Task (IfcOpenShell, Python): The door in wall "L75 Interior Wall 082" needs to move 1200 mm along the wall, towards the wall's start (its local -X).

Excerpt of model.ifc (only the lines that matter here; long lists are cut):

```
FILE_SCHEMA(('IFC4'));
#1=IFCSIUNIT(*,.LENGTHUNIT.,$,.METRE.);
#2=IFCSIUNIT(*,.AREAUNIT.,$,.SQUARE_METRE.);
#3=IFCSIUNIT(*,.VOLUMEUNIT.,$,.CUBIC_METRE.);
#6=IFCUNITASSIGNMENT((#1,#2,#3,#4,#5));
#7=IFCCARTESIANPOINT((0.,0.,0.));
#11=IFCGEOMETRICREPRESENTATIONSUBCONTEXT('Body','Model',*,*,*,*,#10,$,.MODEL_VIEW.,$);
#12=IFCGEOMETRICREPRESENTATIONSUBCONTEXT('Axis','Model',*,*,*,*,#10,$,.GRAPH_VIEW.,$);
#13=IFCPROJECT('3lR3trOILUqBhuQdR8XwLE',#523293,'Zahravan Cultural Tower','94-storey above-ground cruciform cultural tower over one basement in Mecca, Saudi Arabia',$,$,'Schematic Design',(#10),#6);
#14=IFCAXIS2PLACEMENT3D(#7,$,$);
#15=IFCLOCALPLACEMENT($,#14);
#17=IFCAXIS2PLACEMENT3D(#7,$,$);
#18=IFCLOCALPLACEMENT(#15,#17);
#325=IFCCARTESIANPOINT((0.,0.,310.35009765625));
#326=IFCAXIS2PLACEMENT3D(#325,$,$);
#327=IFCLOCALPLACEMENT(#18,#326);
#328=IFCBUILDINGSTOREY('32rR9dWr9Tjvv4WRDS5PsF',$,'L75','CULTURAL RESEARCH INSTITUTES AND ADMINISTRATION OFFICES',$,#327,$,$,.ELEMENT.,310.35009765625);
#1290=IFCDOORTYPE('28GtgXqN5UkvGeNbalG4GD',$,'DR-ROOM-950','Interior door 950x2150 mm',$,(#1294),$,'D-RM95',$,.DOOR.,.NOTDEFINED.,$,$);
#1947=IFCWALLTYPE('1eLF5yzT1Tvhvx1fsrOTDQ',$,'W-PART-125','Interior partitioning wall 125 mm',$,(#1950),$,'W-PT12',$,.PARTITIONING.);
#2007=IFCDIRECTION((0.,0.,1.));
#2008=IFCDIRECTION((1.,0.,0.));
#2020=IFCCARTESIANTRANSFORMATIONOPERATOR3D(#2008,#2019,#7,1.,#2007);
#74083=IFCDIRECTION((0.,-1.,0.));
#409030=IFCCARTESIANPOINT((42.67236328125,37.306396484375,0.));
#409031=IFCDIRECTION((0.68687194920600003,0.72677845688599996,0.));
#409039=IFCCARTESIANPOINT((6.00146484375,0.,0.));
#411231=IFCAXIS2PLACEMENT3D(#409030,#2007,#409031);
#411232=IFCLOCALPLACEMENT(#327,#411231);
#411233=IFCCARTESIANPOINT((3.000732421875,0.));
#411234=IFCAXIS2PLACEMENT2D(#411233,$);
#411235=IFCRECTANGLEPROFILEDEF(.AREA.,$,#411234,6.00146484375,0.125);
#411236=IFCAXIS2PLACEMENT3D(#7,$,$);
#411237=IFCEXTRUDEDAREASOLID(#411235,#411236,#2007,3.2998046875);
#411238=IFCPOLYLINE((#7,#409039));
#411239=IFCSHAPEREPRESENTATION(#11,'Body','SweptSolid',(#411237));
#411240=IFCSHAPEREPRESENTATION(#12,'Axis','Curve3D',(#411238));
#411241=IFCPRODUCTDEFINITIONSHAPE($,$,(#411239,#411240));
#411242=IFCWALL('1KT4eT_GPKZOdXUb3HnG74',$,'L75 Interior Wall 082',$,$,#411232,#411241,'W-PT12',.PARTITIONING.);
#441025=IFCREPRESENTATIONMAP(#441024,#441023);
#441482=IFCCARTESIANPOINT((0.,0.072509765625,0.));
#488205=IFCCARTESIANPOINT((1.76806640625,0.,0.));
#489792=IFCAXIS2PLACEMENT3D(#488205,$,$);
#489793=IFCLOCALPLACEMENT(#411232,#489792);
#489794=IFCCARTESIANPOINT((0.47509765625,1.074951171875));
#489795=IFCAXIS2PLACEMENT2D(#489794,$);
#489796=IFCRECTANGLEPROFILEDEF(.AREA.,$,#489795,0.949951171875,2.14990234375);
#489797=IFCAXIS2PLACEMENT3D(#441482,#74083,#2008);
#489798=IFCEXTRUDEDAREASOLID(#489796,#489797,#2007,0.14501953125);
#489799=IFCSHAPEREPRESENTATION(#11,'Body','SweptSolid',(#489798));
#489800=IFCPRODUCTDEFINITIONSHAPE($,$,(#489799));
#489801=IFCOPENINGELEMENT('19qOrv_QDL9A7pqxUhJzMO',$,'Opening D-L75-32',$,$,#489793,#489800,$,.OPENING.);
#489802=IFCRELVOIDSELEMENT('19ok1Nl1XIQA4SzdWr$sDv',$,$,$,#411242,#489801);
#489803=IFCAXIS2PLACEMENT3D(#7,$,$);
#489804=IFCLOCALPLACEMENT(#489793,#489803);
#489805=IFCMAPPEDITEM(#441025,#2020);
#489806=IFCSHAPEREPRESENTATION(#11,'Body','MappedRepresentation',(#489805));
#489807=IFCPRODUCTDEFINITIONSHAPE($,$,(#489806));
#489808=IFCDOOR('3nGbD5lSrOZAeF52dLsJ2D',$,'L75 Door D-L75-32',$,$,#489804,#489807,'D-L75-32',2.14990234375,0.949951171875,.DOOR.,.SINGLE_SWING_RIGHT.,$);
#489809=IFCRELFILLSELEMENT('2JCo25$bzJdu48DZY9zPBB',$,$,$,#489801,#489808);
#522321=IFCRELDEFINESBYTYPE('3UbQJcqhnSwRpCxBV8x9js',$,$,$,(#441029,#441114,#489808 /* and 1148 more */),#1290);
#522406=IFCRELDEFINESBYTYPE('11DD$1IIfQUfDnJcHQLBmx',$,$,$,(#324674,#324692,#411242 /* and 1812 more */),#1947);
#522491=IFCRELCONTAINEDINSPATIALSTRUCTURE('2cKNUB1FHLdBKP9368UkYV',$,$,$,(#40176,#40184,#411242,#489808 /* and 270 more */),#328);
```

```python
import ifcopenshell
import ifcopenshell.api.geometry
import ifcopenshell.util.placement
import ifcopenshell.util.unit

model = ifcopenshell.open("model.ifc")
unit_scale = ifcopenshell.util.unit.calculate_unit_scale(model)

door = model.by_guid("3nGbD5lSrOZAeF52dLsJ2D")
opening = door.FillsVoids[0].RelatingOpeningElement
wall = opening.VoidsElements[0].RelatingBuildingElement

wall_matrix = ifcopenshell.util.placement.get_local_placement(wall.ObjectPlacement)
shift = wall_matrix[:3, 0] * -1.2 / unit_scale
before = ifcopenshell.util.placement.get_local_placement(door.ObjectPlacement)[:3, 3].copy()

# The door is placed relative to its opening, so it follows when the opening moves.
matrix = ifcopenshell.util.placement.get_local_placement(opening.ObjectPlacement)
matrix[:3, 3] += shift
ifcopenshell.api.geometry.edit_object_placement(
    model, product=opening, matrix=matrix, is_si=False, should_transform_children=True
)

after = ifcopenshell.util.placement.get_local_placement(door.ObjectPlacement)[:3, 3]
print("door moved by", (after - before).round(3) + 0.0)

model.write("model_rev.ifc")
```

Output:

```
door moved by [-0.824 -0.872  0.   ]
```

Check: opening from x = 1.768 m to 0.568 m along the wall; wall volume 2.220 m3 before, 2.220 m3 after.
